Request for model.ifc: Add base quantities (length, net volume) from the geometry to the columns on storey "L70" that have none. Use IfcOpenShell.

First a look at what the model holds.

```python
import ifcopenshell
import ifcopenshell.util.element
import ifcopenshell.util.unit

model = ifcopenshell.open("model.ifc")
print(model.schema)
for unit_type in ("LENGTHUNIT", "AREAUNIT", "VOLUMEUNIT"):
    print(unit_type, ifcopenshell.util.unit.calculate_unit_scale(model, unit_type))
storey = next(s for s in model.by_type("IfcBuildingStorey") if s.Name == "L70")
columns = [e for e in ifcopenshell.util.element.get_decomposition(storey) if e.is_a("IfcColumn")]
for e in sorted(columns, key=lambda e: e.id()):
    print(e.id(), e.is_a(), e.Name, list(ifcopenshell.util.element.get_psets(e, qtos_only=True)), sep=" | ")
```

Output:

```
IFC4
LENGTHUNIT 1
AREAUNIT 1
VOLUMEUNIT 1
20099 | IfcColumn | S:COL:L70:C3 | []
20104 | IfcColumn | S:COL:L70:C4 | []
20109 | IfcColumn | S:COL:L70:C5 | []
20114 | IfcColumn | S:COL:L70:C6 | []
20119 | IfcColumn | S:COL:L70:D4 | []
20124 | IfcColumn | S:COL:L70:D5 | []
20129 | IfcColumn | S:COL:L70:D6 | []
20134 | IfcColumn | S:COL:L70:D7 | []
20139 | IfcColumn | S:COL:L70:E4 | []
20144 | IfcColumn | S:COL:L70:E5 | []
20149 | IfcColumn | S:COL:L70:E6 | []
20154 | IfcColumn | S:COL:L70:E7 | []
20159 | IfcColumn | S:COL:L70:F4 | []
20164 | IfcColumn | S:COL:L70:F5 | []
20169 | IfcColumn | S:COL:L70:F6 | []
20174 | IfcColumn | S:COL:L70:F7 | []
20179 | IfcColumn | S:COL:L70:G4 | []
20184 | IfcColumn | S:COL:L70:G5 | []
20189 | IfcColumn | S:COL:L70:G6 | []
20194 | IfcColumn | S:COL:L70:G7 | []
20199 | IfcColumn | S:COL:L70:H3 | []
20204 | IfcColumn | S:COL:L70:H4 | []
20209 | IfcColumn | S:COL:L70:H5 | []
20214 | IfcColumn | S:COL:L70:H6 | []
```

```python
import ifcopenshell
import ifcopenshell.api.pset
import ifcopenshell.geom
import ifcopenshell.util.element
import ifcopenshell.util.shape
import ifcopenshell.util.unit

model = ifcopenshell.open("model.ifc")
unit_scale = ifcopenshell.util.unit.calculate_unit_scale(model)
volume_scale = ifcopenshell.util.unit.calculate_unit_scale(model, "VOLUMEUNIT")
settings = ifcopenshell.geom.settings()

storey = next(s for s in model.by_type("IfcBuildingStorey") if s.Name == "L70")
columns = [e for e in ifcopenshell.util.element.get_decomposition(storey) if e.is_a("IfcColumn")]

for e in sorted(columns, key=lambda e: e.id()):
    if ifcopenshell.util.element.get_psets(e, qtos_only=True, should_inherit=False):
        continue
    # Geometry comes back in metres, in the element's own axes.
    shape = ifcopenshell.geom.create_shape(settings, e)
    values = {
        "Length": ifcopenshell.util.shape.get_z(shape.geometry) / unit_scale,
        "NetVolume": ifcopenshell.util.shape.get_volume(shape.geometry) / volume_scale,
    }
    qto = ifcopenshell.api.pset.add_qto(model, product=e, name="Qto_ColumnBaseQuantities")
    ifcopenshell.api.pset.edit_qto(model, qto=qto, properties=values)
    print(e.id(), {k: round(v, 3) for k, v in values.items()})

model.write("model_rev.ifc")
```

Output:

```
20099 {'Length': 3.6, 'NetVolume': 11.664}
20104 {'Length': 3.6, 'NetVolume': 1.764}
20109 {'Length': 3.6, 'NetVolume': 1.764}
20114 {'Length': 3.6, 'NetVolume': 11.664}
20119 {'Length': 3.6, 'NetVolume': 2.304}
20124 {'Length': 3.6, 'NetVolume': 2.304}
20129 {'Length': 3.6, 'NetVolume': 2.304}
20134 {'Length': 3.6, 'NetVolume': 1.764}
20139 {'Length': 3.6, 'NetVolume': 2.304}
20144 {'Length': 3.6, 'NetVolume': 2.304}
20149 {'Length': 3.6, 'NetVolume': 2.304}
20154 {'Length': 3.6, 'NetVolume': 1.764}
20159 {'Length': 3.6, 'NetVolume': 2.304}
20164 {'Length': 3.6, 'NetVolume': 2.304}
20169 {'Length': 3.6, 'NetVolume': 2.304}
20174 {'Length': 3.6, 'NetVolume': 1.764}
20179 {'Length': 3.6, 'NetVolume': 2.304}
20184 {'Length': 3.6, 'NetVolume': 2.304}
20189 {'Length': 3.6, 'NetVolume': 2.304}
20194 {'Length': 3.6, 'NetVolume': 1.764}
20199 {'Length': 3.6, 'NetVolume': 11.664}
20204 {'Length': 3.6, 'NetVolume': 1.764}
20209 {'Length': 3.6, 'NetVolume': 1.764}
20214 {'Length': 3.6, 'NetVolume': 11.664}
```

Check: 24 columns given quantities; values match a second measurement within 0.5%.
